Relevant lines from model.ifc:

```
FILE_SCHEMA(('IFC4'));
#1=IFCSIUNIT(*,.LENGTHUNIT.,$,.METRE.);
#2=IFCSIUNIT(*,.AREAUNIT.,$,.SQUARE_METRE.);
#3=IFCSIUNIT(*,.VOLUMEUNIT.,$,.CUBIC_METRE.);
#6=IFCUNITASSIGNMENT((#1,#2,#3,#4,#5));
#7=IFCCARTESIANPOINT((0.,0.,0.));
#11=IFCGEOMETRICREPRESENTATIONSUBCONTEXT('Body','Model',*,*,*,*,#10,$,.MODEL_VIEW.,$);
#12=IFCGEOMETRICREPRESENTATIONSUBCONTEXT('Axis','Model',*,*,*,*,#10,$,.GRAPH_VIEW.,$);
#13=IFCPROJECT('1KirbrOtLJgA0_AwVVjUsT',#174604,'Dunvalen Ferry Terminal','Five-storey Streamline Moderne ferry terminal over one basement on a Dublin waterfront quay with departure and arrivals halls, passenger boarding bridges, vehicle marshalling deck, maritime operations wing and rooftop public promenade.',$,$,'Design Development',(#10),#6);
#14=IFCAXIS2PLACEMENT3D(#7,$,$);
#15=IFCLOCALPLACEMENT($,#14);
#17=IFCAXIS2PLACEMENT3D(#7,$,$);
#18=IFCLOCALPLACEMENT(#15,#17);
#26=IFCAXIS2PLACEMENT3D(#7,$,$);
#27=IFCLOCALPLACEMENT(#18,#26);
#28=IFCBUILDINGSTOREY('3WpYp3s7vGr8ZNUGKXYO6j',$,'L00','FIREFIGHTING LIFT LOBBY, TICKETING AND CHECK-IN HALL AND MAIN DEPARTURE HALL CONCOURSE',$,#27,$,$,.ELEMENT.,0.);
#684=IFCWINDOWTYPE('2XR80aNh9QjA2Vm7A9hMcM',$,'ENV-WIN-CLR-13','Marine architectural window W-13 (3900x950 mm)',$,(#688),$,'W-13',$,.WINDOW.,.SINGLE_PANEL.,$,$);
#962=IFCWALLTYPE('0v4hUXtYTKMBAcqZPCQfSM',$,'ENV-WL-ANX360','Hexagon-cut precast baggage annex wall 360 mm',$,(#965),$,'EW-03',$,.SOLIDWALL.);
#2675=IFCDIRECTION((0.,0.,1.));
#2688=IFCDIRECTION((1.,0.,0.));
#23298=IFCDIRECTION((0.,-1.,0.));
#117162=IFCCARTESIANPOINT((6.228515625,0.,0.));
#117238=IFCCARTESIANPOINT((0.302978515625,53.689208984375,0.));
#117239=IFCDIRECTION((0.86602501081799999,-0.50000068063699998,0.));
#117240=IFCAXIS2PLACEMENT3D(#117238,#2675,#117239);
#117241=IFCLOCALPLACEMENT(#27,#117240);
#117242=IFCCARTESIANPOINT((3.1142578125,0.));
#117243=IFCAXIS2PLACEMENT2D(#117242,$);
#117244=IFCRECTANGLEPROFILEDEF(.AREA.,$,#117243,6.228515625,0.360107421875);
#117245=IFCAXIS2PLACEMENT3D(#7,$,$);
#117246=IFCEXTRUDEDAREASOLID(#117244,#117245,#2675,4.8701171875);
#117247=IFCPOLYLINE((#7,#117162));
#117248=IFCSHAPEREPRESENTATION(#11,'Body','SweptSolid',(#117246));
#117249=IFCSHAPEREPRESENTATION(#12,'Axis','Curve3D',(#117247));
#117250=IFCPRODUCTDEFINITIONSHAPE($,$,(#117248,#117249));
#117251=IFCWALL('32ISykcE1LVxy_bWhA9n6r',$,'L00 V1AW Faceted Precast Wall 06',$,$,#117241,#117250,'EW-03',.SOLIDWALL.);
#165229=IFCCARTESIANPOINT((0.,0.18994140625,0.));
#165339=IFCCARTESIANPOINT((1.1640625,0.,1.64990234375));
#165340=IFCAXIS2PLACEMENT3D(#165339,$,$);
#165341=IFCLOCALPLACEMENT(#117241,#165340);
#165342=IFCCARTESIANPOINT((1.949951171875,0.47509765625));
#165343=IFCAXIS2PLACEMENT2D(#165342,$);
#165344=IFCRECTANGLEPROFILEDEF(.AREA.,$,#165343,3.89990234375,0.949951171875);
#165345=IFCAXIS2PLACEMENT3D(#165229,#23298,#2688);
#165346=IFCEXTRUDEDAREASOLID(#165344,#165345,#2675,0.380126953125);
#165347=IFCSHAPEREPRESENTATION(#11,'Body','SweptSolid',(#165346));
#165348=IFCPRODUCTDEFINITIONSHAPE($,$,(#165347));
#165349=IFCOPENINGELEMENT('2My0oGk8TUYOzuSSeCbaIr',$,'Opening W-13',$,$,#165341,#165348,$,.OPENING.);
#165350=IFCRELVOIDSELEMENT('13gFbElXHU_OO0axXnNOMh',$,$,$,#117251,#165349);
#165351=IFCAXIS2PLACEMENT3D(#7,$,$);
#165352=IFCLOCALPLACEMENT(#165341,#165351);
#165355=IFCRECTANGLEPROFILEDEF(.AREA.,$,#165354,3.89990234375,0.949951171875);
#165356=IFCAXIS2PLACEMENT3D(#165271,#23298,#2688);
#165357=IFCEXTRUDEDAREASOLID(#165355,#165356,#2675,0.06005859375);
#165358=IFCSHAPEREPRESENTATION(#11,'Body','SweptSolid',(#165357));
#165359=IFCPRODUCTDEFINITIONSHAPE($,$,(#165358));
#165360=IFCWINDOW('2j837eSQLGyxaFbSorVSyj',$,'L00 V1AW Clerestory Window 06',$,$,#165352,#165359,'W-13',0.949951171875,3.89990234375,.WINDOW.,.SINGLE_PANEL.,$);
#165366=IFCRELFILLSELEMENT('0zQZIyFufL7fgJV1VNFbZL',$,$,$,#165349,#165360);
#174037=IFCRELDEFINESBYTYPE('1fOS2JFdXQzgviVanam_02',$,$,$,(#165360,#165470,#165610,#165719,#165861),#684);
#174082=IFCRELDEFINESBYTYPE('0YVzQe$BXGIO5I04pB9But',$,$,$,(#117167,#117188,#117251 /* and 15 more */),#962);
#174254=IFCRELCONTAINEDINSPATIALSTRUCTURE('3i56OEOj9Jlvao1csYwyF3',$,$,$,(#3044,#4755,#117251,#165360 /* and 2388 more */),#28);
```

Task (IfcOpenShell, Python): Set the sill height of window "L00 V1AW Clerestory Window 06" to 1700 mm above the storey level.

```python
import numpy as np
import ifcopenshell
import ifcopenshell.api.geometry
import ifcopenshell.geom
import ifcopenshell.util.element
import ifcopenshell.util.placement
import ifcopenshell.util.shape
import ifcopenshell.util.unit

model = ifcopenshell.open("model.ifc")
unit_scale = ifcopenshell.util.unit.calculate_unit_scale(model)

window = model.by_guid("2j837eSQLGyxaFbSorVSyj")
opening = window.FillsVoids[0].RelatingOpeningElement
storey = ifcopenshell.util.element.get_container(window, ifc_class="IfcBuildingStorey")
level = ifcopenshell.util.placement.get_local_placement(storey.ObjectPlacement)[2, 3]

# The opening's origin need not be at the sill, so measure its lowest point.
shape = ifcopenshell.geom.create_shape(ifcopenshell.geom.settings(), opening)
bottom = ifcopenshell.util.shape.get_shape_bottom_elevation(shape, shape.geometry) / unit_scale
dz = level + 1.7 / unit_scale - bottom

shift = np.array([0.0, 0.0, dz])
# The window is placed relative to its opening, so it follows when the opening moves.
matrix = ifcopenshell.util.placement.get_local_placement(opening.ObjectPlacement)
matrix[:3, 3] += shift
ifcopenshell.api.geometry.edit_object_placement(
    model, product=opening, matrix=matrix, is_si=False, should_transform_children=True
)

print(f"moved by {dz * unit_scale:+.3f} m")

model.write("model_v2.ifc")
```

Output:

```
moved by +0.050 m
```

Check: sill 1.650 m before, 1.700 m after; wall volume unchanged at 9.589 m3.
